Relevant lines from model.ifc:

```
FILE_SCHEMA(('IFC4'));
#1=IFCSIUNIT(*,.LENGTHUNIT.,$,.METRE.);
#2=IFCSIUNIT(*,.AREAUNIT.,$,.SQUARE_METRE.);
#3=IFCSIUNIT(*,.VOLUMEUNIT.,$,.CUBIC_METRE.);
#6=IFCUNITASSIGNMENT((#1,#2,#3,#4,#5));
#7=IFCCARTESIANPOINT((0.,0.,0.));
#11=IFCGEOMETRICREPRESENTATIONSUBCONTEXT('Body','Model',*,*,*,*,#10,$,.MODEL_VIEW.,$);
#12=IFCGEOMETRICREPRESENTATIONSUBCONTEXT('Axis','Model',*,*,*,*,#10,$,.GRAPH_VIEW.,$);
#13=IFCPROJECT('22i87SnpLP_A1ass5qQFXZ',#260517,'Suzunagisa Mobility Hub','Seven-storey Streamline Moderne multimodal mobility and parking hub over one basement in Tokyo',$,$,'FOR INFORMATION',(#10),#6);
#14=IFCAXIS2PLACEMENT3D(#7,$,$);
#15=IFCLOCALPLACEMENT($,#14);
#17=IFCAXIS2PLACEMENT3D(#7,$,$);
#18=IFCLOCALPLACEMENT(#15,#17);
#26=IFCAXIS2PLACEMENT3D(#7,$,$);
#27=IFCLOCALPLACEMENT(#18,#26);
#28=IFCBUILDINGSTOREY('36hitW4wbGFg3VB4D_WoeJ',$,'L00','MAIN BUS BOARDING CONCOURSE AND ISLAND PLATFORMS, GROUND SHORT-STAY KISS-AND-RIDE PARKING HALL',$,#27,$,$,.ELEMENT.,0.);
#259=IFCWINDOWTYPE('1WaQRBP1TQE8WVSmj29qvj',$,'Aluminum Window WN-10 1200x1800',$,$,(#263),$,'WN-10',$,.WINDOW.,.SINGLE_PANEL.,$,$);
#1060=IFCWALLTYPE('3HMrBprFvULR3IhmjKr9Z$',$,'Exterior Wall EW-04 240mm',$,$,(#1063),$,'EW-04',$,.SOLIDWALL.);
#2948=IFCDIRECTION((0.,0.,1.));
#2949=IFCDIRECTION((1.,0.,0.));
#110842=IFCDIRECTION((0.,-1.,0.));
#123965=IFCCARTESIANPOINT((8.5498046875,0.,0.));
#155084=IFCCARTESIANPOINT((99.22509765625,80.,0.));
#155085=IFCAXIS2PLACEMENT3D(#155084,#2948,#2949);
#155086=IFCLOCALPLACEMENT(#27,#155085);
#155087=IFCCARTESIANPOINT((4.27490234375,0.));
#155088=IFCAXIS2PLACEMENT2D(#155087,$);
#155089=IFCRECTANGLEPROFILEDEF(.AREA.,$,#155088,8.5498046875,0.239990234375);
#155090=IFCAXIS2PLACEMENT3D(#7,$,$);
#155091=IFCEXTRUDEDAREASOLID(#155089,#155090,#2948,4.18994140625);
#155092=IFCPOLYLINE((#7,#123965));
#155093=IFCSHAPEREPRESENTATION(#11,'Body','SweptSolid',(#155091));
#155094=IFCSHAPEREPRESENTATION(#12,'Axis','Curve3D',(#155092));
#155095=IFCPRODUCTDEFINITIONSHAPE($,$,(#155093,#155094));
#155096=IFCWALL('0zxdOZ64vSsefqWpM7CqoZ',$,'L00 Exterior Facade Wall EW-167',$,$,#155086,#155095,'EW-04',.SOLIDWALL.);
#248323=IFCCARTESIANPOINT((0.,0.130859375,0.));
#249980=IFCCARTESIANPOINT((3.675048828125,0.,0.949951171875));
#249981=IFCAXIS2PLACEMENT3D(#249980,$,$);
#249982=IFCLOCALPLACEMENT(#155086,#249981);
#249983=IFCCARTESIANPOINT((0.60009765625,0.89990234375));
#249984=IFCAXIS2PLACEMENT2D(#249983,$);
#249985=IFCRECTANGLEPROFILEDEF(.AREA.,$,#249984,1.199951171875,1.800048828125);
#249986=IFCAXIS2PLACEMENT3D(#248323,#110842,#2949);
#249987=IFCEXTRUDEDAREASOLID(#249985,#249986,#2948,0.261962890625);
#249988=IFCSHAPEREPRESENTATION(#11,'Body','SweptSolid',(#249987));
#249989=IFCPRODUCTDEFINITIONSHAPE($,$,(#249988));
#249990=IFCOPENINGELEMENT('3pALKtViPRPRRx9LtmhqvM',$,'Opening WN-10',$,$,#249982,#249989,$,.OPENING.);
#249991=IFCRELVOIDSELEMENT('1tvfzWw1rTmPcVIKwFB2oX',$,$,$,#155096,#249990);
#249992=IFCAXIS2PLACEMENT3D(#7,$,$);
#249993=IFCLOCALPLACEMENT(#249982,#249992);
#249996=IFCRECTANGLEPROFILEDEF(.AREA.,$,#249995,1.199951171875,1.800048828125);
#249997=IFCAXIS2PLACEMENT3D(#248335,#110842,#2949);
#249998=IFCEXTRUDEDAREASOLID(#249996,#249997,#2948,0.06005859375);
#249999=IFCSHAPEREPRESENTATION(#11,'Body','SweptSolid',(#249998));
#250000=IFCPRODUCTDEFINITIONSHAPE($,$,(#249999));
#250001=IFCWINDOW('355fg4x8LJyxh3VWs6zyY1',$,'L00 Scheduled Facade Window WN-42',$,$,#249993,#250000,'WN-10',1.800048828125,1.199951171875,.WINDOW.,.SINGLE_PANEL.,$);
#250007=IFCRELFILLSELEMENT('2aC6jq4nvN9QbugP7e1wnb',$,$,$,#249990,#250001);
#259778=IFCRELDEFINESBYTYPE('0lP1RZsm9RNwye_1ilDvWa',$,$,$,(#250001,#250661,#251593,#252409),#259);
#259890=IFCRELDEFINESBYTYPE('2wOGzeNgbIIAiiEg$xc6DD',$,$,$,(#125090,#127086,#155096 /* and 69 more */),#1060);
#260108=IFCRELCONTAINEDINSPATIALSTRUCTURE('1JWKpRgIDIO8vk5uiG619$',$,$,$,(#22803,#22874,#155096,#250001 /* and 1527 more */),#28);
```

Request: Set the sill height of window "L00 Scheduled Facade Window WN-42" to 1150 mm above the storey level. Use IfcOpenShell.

```python
import numpy as np
import ifcopenshell
import ifcopenshell.api.geometry
import ifcopenshell.geom
import ifcopenshell.util.element
import ifcopenshell.util.placement
import ifcopenshell.util.shape
import ifcopenshell.util.unit

model = ifcopenshell.open("model.ifc")
unit_scale = ifcopenshell.util.unit.calculate_unit_scale(model)

window = model.by_guid("355fg4x8LJyxh3VWs6zyY1")
opening = window.FillsVoids[0].RelatingOpeningElement
storey = ifcopenshell.util.element.get_container(window, ifc_class="IfcBuildingStorey")
level = ifcopenshell.util.placement.get_local_placement(storey.ObjectPlacement)[2, 3]

# The opening's origin need not be at the sill, so measure its lowest point.
shape = ifcopenshell.geom.create_shape(ifcopenshell.geom.settings(), opening)
bottom = ifcopenshell.util.shape.get_shape_bottom_elevation(shape, shape.geometry) / unit_scale
dz = level + 1.15 / unit_scale - bottom

shift = np.array([0.0, 0.0, dz])
# The window is placed relative to its opening, so it follows when the opening moves.
matrix = ifcopenshell.util.placement.get_local_placement(opening.ObjectPlacement)
matrix[:3, 3] += shift
ifcopenshell.api.geometry.edit_object_placement(
    model, product=opening, matrix=matrix, is_si=False, should_transform_children=True
)

print(f"moved by {dz * unit_scale:+.3f} m")

model.write("model-out.ifc")
```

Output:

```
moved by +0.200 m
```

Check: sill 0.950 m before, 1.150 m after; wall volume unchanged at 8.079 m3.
